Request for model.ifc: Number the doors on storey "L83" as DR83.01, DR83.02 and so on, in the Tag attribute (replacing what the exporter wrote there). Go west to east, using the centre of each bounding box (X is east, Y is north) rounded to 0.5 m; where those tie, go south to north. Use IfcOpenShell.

First a look at what the model holds.

```python
import ifcopenshell
import ifcopenshell.util.element
import ifcopenshell.util.placement

model = ifcopenshell.open("model.ifc")
print(model.schema)
storey = next(s for s in model.by_type("IfcBuildingStorey") if s.Name == "L83")
doors = [e for e in ifcopenshell.util.element.get_decomposition(storey) if e.is_a("IfcDoor")]
for e in sorted(doors, key=lambda e: e.id()):
    origin = ifcopenshell.util.placement.get_local_placement(e.ObjectPlacement)[:3, 3]
    print(e.id(), e.Tag, e.Name, origin.round(2) + 0.0, sep=" | ")
```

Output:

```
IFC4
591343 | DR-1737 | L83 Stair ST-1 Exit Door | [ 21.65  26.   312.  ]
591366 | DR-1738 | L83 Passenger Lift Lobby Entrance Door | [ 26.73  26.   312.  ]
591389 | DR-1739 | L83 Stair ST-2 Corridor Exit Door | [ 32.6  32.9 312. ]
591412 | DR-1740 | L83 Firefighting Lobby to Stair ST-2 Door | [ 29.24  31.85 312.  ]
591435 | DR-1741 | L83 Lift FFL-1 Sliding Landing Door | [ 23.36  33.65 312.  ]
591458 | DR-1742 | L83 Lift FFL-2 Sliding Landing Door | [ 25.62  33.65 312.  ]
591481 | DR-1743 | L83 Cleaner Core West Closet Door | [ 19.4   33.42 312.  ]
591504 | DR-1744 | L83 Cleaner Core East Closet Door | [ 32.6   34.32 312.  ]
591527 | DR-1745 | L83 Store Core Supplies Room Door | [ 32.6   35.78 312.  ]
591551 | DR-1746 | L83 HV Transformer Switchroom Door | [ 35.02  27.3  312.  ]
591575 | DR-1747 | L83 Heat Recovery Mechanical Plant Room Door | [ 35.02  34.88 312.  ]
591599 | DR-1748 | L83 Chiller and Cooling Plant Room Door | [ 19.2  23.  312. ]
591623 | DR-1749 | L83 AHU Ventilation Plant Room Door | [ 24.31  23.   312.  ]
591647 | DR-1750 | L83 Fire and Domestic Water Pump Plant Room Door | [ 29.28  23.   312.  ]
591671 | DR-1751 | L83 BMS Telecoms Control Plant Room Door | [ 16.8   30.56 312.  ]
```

```python
import ifcopenshell
import ifcopenshell.geom
import ifcopenshell.util.element
import ifcopenshell.util.shape

model = ifcopenshell.open("model.ifc")
settings = ifcopenshell.geom.settings()
settings.set("use-world-coords", True)


def centre(element):
    shape = ifcopenshell.geom.create_shape(settings, element)
    return ifcopenshell.util.shape.get_bbox_centroid(shape.geometry)


storey = next(s for s in model.by_type("IfcBuildingStorey") if s.Name == "L83")
doors = [e for e in ifcopenshell.util.element.get_decomposition(storey) if e.is_a("IfcDoor")]

# Insertion points can sit at a corner or the storey origin, so sort by the geometry (in metres).
centres = {e: centre(e) for e in doors}
doors.sort(key=lambda e: (round(centres[e][0] / 0.5), centres[e][1]))

for i, e in enumerate(doors, start=1):
    number = f"DR83.{i:02d}"
    e.Tag = number
    print(e.id(), number)

model.write("model_rev.ifc")
```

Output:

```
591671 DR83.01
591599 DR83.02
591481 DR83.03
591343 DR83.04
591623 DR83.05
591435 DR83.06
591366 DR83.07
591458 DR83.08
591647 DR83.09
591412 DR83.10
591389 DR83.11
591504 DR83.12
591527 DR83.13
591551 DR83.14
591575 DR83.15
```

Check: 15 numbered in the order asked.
